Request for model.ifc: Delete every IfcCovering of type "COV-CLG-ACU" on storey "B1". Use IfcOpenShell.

First a look at what the model holds.

```python
import ifcopenshell
import ifcopenshell.util.element

model = ifcopenshell.open("model.ifc")
print(model.schema)
storey = next(s for s in model.by_type("IfcBuildingStorey") if s.Name == "B1")
coverings = [e for e in ifcopenshell.util.element.get_decomposition(storey) if e.is_a("IfcCovering")]
seen = {}
for e in coverings:
    element_type = ifcopenshell.util.element.get_type(e)
    name = element_type.Name if element_type not in (None, e) else None
    seen[name] = seen.get(name, 0) + 1
for name, count in sorted(seen.items(), key=str):
    print(count, "x", name)
```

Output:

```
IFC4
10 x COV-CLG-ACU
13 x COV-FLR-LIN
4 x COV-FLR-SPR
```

```python
import ifcopenshell
import ifcopenshell.api.root
import ifcopenshell.util.element

model = ifcopenshell.open("model.ifc")

storey = next(s for s in model.by_type("IfcBuildingStorey") if s.Name == "B1")
coverings = [e for e in ifcopenshell.util.element.get_decomposition(storey) if e.is_a("IfcCovering")]
targets = [e for e in coverings if (t := ifcopenshell.util.element.get_type(e)) not in (None, e) and t.Name == "COV-CLG-ACU"]

for e in targets:
    ifcopenshell.api.root.remove_product(model, product=e)
print(len(targets), "removed")

model.write("model_rev.ifc")
```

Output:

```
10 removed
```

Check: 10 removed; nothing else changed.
